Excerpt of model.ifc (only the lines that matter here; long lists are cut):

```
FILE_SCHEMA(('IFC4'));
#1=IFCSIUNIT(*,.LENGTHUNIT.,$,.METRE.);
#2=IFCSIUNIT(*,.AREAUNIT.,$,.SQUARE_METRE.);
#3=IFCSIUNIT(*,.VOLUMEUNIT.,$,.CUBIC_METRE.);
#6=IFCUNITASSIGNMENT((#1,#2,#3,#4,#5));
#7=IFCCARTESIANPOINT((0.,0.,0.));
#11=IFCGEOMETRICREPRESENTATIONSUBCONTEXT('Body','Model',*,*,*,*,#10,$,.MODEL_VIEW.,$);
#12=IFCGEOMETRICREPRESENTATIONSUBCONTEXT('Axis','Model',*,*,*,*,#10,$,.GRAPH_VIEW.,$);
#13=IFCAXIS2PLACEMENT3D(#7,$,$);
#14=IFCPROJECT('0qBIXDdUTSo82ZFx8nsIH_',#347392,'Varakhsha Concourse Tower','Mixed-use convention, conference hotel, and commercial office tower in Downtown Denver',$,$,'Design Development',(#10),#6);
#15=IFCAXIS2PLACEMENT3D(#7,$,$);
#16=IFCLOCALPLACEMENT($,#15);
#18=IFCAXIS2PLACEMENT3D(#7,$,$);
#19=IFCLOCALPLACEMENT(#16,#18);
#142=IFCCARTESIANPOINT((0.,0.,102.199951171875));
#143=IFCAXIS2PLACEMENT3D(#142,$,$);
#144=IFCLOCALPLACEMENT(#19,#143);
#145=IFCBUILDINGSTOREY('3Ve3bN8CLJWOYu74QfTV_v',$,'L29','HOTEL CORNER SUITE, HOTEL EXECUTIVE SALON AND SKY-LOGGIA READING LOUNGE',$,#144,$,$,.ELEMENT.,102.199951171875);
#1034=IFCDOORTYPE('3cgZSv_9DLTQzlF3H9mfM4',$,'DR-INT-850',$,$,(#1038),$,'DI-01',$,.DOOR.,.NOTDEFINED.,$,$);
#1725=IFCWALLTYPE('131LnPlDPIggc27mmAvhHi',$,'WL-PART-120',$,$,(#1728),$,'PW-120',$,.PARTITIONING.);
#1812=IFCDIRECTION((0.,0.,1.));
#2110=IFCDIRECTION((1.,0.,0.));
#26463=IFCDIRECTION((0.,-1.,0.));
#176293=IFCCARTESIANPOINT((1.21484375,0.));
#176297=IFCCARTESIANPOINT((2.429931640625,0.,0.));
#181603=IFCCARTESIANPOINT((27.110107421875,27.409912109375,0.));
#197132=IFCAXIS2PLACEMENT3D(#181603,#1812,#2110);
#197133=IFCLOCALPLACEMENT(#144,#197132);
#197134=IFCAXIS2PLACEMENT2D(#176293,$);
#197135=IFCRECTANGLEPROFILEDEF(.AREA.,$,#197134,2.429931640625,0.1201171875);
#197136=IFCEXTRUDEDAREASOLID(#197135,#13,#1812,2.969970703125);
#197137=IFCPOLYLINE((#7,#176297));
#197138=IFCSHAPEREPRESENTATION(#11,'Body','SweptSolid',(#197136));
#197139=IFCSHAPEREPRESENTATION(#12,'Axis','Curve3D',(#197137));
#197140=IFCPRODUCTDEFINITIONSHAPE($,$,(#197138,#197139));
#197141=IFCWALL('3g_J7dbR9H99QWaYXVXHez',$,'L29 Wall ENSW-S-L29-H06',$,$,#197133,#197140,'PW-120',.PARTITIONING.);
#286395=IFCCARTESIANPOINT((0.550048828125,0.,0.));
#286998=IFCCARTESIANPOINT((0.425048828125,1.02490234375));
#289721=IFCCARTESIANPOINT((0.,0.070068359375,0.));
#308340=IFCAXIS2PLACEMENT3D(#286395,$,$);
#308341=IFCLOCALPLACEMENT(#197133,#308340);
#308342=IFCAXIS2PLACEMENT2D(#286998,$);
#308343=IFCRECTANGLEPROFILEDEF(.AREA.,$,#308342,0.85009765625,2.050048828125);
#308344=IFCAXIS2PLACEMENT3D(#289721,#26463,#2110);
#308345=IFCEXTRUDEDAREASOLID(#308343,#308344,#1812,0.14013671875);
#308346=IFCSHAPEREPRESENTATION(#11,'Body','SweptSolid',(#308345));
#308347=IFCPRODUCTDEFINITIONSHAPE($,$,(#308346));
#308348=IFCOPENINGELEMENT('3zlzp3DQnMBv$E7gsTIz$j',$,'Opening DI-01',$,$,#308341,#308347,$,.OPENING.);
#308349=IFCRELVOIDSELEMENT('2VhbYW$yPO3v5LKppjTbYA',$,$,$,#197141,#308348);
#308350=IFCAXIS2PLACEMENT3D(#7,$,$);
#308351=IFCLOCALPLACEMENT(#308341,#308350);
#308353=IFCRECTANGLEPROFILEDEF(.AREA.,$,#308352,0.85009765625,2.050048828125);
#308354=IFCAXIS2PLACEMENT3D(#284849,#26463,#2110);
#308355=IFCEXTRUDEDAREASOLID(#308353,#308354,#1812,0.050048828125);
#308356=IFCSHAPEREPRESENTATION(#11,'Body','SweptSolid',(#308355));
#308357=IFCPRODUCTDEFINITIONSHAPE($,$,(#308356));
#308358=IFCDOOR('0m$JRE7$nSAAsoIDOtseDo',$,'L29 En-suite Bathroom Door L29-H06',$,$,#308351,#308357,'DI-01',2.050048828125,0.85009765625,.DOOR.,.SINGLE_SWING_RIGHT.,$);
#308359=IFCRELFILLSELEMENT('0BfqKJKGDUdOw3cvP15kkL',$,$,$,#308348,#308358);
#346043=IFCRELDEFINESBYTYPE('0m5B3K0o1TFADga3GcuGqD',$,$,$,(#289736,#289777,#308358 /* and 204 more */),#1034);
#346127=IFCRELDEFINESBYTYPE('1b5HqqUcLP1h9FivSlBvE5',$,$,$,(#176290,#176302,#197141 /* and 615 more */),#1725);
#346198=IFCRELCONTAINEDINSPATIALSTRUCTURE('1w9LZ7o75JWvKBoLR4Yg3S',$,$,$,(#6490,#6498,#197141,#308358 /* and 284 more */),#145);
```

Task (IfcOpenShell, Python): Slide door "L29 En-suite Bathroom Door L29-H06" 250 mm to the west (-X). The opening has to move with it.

```python
import ifcopenshell
import ifcopenshell.api.geometry
import ifcopenshell.util.placement

model = ifcopenshell.open("model.ifc")

door = model.by_guid("0m$JRE7$nSAAsoIDOtseDo")
opening = door.FillsVoids[0].RelatingOpeningElement
wall = opening.VoidsElements[0].RelatingBuildingElement

wall_matrix = ifcopenshell.util.placement.get_local_placement(wall.ObjectPlacement)
shift = wall_matrix[:3, 0] * -0.25
before = ifcopenshell.util.placement.get_local_placement(door.ObjectPlacement)[:3, 3].copy()

# The door is placed relative to its opening, so it follows when the opening moves.
matrix = ifcopenshell.util.placement.get_local_placement(opening.ObjectPlacement)
matrix[:3, 3] += shift
ifcopenshell.api.geometry.edit_object_placement(
    model, product=opening, matrix=matrix, is_si=False, should_transform_children=True
)

after = ifcopenshell.util.placement.get_local_placement(door.ObjectPlacement)[:3, 3]
print("door moved by", (after - before).round(3) + 0.0)

model.write("model_rev.ifc")
```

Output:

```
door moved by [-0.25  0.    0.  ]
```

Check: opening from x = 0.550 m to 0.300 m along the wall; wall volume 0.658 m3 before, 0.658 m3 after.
